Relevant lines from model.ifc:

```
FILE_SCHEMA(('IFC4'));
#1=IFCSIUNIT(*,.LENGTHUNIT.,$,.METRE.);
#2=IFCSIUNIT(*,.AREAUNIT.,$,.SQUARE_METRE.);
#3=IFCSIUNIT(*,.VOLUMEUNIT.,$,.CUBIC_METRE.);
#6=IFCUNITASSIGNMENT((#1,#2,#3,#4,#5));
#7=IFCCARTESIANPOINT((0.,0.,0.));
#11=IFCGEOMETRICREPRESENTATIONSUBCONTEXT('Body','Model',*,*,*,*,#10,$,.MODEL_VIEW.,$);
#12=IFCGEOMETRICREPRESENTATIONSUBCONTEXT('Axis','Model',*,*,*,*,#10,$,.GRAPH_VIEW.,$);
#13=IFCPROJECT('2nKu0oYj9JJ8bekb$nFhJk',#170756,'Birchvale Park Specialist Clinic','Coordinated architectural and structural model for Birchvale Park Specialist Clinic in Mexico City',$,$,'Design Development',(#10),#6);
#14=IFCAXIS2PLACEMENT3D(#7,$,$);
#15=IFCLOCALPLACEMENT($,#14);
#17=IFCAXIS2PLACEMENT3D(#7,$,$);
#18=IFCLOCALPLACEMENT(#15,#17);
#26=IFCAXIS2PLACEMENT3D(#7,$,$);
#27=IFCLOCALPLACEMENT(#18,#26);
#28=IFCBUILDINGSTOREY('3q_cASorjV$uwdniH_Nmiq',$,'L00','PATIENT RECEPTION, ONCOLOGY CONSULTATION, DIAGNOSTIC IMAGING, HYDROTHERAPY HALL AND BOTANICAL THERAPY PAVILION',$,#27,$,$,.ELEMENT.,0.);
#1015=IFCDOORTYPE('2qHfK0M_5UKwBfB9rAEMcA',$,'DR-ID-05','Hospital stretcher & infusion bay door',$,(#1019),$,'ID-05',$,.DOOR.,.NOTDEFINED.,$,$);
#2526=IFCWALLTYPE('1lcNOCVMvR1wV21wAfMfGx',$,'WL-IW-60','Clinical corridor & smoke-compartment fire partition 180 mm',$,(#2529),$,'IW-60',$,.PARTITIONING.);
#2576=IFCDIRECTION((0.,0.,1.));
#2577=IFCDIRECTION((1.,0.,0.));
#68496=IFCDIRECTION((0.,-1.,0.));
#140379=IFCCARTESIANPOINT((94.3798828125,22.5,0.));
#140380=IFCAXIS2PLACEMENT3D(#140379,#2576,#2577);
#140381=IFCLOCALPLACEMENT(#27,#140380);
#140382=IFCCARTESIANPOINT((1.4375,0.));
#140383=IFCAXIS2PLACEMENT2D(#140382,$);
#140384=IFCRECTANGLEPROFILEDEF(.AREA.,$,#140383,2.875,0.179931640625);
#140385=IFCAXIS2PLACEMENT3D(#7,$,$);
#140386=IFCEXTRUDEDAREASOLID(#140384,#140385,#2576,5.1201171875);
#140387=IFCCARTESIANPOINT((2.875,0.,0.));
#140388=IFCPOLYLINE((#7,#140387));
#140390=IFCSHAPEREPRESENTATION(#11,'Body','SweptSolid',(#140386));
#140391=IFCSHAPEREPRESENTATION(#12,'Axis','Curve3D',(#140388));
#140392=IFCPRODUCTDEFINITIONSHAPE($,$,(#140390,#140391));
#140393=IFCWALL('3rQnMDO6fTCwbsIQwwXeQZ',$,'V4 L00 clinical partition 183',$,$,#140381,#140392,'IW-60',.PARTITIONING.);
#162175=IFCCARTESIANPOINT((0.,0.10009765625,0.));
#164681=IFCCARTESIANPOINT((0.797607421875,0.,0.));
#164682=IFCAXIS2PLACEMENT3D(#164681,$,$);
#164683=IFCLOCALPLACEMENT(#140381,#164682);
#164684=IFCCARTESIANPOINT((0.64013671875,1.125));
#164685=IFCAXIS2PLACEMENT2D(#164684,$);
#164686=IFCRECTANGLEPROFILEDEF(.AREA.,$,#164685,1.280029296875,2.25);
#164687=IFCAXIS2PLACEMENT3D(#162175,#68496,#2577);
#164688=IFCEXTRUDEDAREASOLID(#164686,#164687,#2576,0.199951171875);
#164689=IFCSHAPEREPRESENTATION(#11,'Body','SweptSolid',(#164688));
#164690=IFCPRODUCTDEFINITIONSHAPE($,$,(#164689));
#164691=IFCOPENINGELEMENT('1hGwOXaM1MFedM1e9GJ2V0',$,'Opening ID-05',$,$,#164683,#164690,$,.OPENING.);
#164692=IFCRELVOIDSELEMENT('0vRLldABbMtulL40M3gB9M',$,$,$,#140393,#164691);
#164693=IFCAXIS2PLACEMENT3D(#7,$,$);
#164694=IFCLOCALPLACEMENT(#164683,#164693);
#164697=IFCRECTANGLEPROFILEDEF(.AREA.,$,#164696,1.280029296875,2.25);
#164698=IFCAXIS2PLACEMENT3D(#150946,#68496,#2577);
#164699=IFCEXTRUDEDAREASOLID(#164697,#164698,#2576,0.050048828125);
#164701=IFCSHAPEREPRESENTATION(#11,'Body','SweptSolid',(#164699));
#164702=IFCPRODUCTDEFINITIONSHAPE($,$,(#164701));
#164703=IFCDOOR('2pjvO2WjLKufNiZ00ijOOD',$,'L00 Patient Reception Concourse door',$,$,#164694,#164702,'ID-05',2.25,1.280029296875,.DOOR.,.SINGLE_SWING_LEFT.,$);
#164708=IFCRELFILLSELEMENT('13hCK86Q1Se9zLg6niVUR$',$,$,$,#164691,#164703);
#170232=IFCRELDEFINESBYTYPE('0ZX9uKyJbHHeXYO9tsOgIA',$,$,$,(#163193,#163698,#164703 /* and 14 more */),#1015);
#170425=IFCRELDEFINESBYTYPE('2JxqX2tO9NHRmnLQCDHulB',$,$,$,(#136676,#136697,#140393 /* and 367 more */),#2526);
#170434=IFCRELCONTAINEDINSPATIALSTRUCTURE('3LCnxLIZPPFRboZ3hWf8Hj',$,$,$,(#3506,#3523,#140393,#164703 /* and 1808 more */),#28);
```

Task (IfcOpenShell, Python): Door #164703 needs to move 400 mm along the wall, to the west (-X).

```python
import ifcopenshell
import ifcopenshell.api.geometry
import ifcopenshell.util.placement
import ifcopenshell.util.unit

model = ifcopenshell.open("model.ifc")
unit_scale = ifcopenshell.util.unit.calculate_unit_scale(model)

door = model.by_guid("2pjvO2WjLKufNiZ00ijOOD")
opening = door.FillsVoids[0].RelatingOpeningElement
wall = opening.VoidsElements[0].RelatingBuildingElement

wall_matrix = ifcopenshell.util.placement.get_local_placement(wall.ObjectPlacement)
shift = wall_matrix[:3, 0] * -0.4 / unit_scale
before = ifcopenshell.util.placement.get_local_placement(door.ObjectPlacement)[:3, 3].copy()

# The door is placed relative to its opening, so it follows when the opening moves.
matrix = ifcopenshell.util.placement.get_local_placement(opening.ObjectPlacement)
matrix[:3, 3] += shift
ifcopenshell.api.geometry.edit_object_placement(
    model, product=opening, matrix=matrix, is_si=False, should_transform_children=True
)

after = ifcopenshell.util.placement.get_local_placement(door.ObjectPlacement)[:3, 3]
print("door moved by", (after - before).round(3) + 0.0)

model.write("model-out.ifc")
```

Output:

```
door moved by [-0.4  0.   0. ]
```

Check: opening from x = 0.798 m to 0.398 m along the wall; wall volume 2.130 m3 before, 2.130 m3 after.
